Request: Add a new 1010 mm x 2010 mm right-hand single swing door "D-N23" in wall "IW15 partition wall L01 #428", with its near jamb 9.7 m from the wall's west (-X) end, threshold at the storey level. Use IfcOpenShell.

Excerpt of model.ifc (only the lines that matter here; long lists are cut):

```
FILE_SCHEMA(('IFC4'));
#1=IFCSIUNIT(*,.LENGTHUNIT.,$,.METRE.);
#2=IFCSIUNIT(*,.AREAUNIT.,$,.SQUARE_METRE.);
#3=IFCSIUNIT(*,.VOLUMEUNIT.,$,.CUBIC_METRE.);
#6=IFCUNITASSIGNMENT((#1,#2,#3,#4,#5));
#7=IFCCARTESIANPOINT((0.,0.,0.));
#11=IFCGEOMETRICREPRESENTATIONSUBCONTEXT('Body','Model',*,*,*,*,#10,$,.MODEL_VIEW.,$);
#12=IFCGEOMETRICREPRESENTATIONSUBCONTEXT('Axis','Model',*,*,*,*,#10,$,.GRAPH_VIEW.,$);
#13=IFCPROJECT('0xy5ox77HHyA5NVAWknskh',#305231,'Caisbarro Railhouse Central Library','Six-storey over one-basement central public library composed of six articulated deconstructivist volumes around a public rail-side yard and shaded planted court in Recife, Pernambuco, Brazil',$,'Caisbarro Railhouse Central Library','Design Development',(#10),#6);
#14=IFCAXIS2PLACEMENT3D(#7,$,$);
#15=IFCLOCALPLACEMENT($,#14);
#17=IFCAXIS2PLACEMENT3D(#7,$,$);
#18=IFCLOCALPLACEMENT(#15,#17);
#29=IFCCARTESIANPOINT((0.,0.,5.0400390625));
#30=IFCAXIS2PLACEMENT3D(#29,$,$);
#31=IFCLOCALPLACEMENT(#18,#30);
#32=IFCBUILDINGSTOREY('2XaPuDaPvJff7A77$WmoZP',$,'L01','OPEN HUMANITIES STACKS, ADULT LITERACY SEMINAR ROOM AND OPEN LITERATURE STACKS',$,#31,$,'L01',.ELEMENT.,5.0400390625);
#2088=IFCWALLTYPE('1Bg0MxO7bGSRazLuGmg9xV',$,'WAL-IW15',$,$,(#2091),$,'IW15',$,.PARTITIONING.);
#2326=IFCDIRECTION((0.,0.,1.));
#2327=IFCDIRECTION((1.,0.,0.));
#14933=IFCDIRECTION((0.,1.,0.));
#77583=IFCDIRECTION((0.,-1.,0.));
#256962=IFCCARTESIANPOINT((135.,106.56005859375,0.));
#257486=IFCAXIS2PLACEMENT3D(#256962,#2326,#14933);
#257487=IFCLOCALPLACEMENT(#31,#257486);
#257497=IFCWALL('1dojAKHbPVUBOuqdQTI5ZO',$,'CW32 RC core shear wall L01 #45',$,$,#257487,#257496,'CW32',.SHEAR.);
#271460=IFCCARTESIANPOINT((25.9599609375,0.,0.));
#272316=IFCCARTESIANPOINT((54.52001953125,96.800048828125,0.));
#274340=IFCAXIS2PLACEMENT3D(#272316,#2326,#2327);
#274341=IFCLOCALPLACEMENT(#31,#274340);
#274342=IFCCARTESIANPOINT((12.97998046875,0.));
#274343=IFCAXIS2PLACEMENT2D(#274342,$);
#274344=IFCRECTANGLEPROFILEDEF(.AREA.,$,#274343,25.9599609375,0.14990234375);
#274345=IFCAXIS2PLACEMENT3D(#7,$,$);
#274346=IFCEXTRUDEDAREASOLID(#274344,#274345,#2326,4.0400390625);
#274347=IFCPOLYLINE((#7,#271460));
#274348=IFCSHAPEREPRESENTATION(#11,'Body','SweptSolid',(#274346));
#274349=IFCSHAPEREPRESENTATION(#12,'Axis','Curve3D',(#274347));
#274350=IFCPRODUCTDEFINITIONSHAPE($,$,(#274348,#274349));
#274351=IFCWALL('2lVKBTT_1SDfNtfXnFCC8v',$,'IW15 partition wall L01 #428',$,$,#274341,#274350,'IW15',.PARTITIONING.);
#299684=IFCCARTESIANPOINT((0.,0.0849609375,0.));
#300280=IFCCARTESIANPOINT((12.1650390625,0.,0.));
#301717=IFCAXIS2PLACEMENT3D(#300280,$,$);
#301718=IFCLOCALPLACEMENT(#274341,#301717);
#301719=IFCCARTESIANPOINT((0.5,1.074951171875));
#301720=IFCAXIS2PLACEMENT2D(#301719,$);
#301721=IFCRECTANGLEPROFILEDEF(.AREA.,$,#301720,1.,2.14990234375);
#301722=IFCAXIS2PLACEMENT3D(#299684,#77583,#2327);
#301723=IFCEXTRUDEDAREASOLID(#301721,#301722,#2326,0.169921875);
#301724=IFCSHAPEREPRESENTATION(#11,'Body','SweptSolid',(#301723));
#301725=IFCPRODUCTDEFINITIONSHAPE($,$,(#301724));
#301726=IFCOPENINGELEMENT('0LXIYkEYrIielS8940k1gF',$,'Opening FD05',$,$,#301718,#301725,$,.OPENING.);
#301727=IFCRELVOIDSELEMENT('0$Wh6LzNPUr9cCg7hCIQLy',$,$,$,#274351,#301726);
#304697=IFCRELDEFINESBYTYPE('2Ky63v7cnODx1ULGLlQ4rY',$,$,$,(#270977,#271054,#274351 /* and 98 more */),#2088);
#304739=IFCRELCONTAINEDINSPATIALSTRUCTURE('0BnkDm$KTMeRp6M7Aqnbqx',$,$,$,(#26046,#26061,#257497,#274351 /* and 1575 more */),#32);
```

```python
import numpy as np
import ifcopenshell
import ifcopenshell.api.feature
import ifcopenshell.api.geometry
import ifcopenshell.api.root
import ifcopenshell.api.spatial
import ifcopenshell.geom
import ifcopenshell.util.element
import ifcopenshell.util.placement
import ifcopenshell.util.representation
import ifcopenshell.util.shape
import ifcopenshell.util.unit

model = ifcopenshell.open("model.ifc")
unit_scale = ifcopenshell.util.unit.calculate_unit_scale(model)
settings = ifcopenshell.geom.settings()


def volume(element):
    """Net volume in cubic metres, openings subtracted."""
    shape = ifcopenshell.geom.create_shape(settings, element)
    return ifcopenshell.util.shape.get_volume(shape.geometry)


wall = model.by_guid("2lVKBTT_1SDfNtfXnFCC8v")
storey = ifcopenshell.util.element.get_container(wall, ifc_class="IfcBuildingStorey")
context = ifcopenshell.util.representation.get_context(model, "Model", "Body", "MODEL_VIEW")
before = volume(wall)

width, height, from_end, sill = 1.01, 2.01, 9.7, 0.0  # metres

# The wall runs along its own X axis, and the end named is its -X end.
wall_shape = ifcopenshell.geom.create_shape(settings, wall)
x, y, z = ifcopenshell.util.shape.get_vertices(wall_shape.geometry).T
start = x.min() + from_end
face, thickness = float(y.min()), float(y.max() - y.min())
wall_matrix = ifcopenshell.util.placement.get_local_placement(wall.ObjectPlacement)
level = ifcopenshell.util.placement.get_local_placement(storey.ObjectPlacement)[2, 3]


def in_wall(x, y):
    """Placement at x, y metres in the wall's axes, at sill height."""
    matrix = wall_matrix.copy()
    matrix[:, 3] = wall_matrix @ np.array([x / unit_scale, y / unit_scale, 0.0, 1.0])
    matrix[2, 3] = level + sill / unit_scale
    return matrix


# Opening: a box that overshoots both wall faces by 50 mm.
opening = ifcopenshell.api.root.create_entity(model, ifc_class="IfcOpeningElement", predefined_type="OPENING")
box = ifcopenshell.api.geometry.add_wall_representation(
    model, context=context, length=width, height=height, thickness=thickness + 0.1
)
ifcopenshell.api.geometry.assign_representation(model, product=opening, representation=box)
ifcopenshell.api.geometry.edit_object_placement(model, product=opening, matrix=in_wall(start, face - 0.05), is_si=False)
ifcopenshell.api.feature.add_feature(model, feature=opening, element=wall)

door = ifcopenshell.api.root.create_entity(model, ifc_class="IfcDoor", name="D-N23", predefined_type="DOOR")
door.OverallWidth, door.OverallHeight = width / unit_scale, height / unit_scale
door.OperationType = "SINGLE_SWING_RIGHT"
body = ifcopenshell.api.geometry.add_door_representation(
    model,
    context=context,
    overall_width=door.OverallWidth,
    overall_height=door.OverallHeight,
    operation_type="SINGLE_SWING_RIGHT",
    lining_properties={"LiningDepth": thickness / unit_scale, "ThresholdDepth": thickness / unit_scale},
)
ifcopenshell.api.geometry.assign_representation(model, product=door, representation=body)
ifcopenshell.api.spatial.assign_container(model, products=[door], relating_structure=storey)
ifcopenshell.api.feature.add_filling(model, opening=opening, element=door)

# The lining spans the wall, so the door starts at the wall face.
ifcopenshell.api.geometry.edit_object_placement(model, product=door, matrix=in_wall(start, face), is_si=False)

after = volume(wall)

print(f"wall volume {before:.3f} -> {after:.3f} m3")

model.write("model_edited.ifc")
```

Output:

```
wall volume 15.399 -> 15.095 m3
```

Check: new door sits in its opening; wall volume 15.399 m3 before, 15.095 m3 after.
